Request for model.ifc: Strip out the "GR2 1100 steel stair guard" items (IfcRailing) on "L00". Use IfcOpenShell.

First a look at what the model holds.

```python
import ifcopenshell
import ifcopenshell.util.element

model = ifcopenshell.open("model.ifc")
print(model.schema)
storey = next(s for s in model.by_type("IfcBuildingStorey") if s.Name == "L00")
railings = [e for e in ifcopenshell.util.element.get_decomposition(storey) if e.is_a("IfcRailing")]
seen = {}
for e in railings:
    element_type = ifcopenshell.util.element.get_type(e)
    name = element_type.Name if element_type not in (None, e) else None
    seen[name] = seen.get(name, 0) + 1
for name, count in sorted(seen.items(), key=str):
    print(count, "x", name)
```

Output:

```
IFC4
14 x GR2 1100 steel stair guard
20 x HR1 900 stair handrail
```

```python
import ifcopenshell
import ifcopenshell.api.root
import ifcopenshell.util.element

model = ifcopenshell.open("model.ifc")

storey = next(s for s in model.by_type("IfcBuildingStorey") if s.Name == "L00")
railings = [e for e in ifcopenshell.util.element.get_decomposition(storey) if e.is_a("IfcRailing")]
targets = [e for e in railings if (t := ifcopenshell.util.element.get_type(e)) not in (None, e) and t.Name == "GR2 1100 steel stair guard"]

for e in targets:
    ifcopenshell.api.root.remove_product(model, product=e)
print(len(targets), "removed")

model.write("model_updated.ifc")
```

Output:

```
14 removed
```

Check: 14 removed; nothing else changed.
